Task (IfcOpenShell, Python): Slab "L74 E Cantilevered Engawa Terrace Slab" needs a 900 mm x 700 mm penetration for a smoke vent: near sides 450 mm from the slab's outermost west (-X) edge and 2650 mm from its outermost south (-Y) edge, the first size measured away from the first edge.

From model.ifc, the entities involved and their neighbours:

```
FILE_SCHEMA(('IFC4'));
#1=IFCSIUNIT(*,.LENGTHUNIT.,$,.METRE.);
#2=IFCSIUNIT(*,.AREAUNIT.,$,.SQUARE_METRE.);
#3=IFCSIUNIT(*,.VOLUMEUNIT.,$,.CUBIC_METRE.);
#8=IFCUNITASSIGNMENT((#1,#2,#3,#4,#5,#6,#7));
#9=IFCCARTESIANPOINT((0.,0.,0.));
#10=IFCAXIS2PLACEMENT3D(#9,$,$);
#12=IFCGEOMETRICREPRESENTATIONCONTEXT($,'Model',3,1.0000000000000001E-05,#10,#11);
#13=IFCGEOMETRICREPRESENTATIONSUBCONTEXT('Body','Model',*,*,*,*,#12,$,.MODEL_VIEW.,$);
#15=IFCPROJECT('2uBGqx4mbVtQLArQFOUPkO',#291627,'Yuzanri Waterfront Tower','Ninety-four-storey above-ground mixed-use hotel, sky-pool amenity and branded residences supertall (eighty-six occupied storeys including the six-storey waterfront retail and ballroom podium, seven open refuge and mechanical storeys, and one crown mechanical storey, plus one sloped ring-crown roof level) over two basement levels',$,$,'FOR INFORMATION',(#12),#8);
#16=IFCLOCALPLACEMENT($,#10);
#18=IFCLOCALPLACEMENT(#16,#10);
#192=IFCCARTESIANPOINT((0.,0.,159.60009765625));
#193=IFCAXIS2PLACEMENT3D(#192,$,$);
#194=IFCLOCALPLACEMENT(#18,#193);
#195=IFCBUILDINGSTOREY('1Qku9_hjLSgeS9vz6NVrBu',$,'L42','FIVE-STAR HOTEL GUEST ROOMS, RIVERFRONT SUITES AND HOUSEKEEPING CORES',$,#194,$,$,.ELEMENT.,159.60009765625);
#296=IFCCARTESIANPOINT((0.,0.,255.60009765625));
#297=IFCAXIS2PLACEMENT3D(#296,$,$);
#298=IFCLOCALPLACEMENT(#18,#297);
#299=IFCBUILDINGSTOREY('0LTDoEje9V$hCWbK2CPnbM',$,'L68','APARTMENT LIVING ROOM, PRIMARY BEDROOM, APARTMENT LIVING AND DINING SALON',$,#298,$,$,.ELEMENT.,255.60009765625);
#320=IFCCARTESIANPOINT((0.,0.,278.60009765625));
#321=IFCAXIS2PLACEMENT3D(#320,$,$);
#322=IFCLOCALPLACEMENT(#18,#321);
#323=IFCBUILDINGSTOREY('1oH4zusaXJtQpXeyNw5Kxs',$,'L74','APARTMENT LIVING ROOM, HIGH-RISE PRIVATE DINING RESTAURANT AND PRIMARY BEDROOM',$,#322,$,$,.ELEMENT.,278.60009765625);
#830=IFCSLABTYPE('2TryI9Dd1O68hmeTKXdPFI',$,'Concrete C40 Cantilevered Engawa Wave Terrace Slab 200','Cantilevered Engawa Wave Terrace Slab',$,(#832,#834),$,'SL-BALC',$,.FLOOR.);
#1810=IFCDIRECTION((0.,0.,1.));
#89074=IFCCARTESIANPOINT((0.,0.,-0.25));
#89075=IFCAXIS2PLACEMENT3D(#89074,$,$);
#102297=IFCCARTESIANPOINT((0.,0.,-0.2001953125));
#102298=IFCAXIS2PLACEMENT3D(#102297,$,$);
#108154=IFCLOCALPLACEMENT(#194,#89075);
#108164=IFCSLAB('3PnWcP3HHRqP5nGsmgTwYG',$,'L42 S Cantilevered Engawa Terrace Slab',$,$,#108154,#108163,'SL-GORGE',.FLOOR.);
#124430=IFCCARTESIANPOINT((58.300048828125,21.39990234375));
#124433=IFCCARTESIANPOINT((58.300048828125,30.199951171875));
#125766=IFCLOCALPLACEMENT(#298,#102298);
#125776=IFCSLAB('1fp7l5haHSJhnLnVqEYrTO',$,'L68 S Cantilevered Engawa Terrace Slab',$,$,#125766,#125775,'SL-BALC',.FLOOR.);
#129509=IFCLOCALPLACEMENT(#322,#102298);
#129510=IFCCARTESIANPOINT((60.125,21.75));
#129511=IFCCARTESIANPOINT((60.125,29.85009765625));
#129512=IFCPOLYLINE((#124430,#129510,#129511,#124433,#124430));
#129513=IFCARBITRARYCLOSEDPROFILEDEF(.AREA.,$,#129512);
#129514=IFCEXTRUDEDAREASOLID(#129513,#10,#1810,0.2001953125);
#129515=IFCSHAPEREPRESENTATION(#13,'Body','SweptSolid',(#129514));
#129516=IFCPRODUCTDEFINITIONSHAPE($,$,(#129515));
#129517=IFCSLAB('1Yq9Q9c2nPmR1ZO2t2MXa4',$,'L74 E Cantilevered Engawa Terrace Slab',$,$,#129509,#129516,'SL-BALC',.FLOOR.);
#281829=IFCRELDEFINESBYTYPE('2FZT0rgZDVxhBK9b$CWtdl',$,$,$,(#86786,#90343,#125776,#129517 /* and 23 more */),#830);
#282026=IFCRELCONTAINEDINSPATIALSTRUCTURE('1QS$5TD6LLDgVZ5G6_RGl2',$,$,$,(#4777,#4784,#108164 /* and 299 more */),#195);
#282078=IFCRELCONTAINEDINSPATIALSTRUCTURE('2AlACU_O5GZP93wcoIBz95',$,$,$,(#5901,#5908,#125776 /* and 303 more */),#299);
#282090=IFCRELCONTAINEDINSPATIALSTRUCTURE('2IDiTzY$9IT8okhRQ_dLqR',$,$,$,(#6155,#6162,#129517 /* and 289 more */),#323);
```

```python
import numpy as np
import ifcopenshell
import ifcopenshell.api.feature
import ifcopenshell.api.geometry
import ifcopenshell.api.root
import ifcopenshell.geom
import ifcopenshell.util.placement
import ifcopenshell.util.representation
import ifcopenshell.util.shape
import ifcopenshell.util.unit

model = ifcopenshell.open("model.ifc")
unit_scale = ifcopenshell.util.unit.calculate_unit_scale(model)
settings = ifcopenshell.geom.settings()


def volume(element):
    """Net volume in cubic metres, openings subtracted."""
    shape = ifcopenshell.geom.create_shape(settings, element)
    return ifcopenshell.util.shape.get_volume(shape.geometry)


slab = model.by_guid("1Yq9Q9c2nPmR1ZO2t2MXa4")
before = volume(slab)

# Extent in the slab's own axes, in metres. The edges named are its -X and -Y sides.
slab_shape = ifcopenshell.geom.create_shape(settings, slab)
vertices = ifcopenshell.util.shape.get_vertices(slab_shape.geometry)
x_min, y_min, bottom = vertices.min(axis=0)
top = vertices[:, 2].max()

opening = ifcopenshell.api.root.create_entity(model, ifc_class="IfcOpeningElement", name="Smoke vent opening", predefined_type="OPENING")
context = ifcopenshell.util.representation.get_context(model, "Model", "Body", "MODEL_VIEW")
width, depth = 0.9, 0.7
outline = [(0.0, 0.0), (width, 0.0), (width, depth), (0.0, depth), (0.0, 0.0)]
# Overshoot both faces by 50 mm so the cut is clean.
shape = ifcopenshell.api.geometry.add_slab_representation(
    model, context=context, depth=top - bottom + 0.1, polyline=outline
)
ifcopenshell.api.geometry.assign_representation(model, product=opening, representation=shape)

matrix = ifcopenshell.util.placement.get_local_placement(slab.ObjectPlacement)
matrix[:, 3] = matrix @ np.append(np.array([x_min + 0.45, y_min + 2.65, bottom - 0.05]) / unit_scale, 1.0)
ifcopenshell.api.geometry.edit_object_placement(model, product=opening, matrix=matrix, is_si=False)
ifcopenshell.api.feature.add_feature(model, feature=opening, element=slab)

after = volume(slab)

print(f"slab volume {before:.3f} -> {after:.3f} m3")

model.write("model_edited.ifc")
```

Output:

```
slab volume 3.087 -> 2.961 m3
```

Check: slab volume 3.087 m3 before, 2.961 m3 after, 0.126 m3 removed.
